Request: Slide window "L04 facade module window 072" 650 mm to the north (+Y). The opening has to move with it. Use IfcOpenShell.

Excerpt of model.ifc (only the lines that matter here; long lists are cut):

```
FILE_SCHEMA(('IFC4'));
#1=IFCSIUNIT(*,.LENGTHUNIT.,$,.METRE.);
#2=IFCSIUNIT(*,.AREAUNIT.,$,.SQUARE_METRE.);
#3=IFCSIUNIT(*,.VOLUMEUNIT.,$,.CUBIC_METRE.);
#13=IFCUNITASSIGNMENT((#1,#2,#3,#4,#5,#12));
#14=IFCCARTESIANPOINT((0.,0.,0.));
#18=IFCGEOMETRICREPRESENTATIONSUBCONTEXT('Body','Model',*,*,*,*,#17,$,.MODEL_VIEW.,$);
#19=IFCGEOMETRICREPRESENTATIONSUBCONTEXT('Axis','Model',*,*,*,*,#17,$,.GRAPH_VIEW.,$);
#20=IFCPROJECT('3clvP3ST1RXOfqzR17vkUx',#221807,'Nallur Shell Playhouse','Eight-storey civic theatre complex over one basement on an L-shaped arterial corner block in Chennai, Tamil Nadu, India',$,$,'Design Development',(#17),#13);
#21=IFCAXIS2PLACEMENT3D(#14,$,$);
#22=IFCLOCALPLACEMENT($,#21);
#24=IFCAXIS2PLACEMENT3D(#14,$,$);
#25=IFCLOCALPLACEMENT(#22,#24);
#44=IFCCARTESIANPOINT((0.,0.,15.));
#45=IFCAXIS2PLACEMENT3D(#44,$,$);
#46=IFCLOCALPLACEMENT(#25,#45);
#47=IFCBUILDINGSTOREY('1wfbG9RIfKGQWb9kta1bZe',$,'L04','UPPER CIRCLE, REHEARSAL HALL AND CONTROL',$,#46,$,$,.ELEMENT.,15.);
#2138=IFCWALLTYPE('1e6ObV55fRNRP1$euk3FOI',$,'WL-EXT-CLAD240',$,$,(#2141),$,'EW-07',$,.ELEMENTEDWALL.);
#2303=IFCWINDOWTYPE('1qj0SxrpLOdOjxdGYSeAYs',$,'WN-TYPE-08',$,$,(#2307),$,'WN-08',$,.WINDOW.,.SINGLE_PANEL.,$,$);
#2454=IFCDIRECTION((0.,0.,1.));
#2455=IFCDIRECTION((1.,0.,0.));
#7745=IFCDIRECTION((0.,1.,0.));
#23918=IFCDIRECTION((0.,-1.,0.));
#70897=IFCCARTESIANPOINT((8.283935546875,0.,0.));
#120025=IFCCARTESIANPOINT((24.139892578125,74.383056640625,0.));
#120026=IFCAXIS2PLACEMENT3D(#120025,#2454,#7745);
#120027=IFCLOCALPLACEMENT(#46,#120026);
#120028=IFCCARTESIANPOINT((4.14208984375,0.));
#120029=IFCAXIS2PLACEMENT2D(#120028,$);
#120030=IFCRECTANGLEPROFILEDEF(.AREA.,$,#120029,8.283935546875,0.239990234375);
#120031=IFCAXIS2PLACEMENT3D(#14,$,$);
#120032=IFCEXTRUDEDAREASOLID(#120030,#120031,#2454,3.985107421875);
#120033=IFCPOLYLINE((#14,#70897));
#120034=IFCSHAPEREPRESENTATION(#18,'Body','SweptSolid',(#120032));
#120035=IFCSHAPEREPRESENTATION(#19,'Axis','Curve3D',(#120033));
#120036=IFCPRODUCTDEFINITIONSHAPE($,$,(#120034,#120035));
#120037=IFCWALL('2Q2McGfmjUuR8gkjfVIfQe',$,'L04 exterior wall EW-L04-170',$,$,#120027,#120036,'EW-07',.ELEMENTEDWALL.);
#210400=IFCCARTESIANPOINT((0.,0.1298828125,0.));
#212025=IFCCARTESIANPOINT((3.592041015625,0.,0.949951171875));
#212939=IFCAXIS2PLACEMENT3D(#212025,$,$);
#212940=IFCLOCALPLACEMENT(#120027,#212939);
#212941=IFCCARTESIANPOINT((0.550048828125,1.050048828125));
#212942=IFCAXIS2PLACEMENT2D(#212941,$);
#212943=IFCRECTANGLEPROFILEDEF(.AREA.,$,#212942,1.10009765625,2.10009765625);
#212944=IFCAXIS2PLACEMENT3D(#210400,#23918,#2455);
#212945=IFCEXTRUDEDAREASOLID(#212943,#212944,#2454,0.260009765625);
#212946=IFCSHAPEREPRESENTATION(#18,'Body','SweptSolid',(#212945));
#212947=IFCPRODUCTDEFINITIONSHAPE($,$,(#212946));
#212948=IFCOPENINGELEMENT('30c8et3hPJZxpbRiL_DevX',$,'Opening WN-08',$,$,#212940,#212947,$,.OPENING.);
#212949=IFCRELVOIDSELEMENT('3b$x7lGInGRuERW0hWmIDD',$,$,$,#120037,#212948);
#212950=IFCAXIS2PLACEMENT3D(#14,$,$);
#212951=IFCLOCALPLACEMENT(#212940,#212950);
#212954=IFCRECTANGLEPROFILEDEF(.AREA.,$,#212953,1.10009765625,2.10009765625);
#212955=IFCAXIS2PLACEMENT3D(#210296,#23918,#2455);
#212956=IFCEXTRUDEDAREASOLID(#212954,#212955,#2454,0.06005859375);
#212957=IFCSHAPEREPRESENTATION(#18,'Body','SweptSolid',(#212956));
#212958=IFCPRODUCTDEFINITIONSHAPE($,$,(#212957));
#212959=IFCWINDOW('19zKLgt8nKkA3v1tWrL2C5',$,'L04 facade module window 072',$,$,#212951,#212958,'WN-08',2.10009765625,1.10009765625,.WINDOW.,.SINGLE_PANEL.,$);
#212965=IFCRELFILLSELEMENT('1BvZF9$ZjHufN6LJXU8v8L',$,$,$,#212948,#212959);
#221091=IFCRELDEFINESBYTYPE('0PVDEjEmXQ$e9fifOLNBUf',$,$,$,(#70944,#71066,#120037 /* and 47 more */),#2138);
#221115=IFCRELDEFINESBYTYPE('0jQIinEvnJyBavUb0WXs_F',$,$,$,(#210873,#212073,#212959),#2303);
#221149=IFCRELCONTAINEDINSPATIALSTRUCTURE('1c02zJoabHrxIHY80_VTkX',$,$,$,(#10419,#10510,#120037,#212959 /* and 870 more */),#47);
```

```python
import ifcopenshell
import ifcopenshell.api.geometry
import ifcopenshell.util.placement

model = ifcopenshell.open("model.ifc")

window = model.by_id(212959)
opening = window.FillsVoids[0].RelatingOpeningElement
wall = opening.VoidsElements[0].RelatingBuildingElement

wall_matrix = ifcopenshell.util.placement.get_local_placement(wall.ObjectPlacement)
shift = wall_matrix[:3, 0] * 0.65
before = ifcopenshell.util.placement.get_local_placement(window.ObjectPlacement)[:3, 3].copy()

# The window is placed relative to its opening, so it follows when the opening moves.
matrix = ifcopenshell.util.placement.get_local_placement(opening.ObjectPlacement)
matrix[:3, 3] += shift
ifcopenshell.api.geometry.edit_object_placement(
    model, product=opening, matrix=matrix, is_si=False, should_transform_children=True
)

after = ifcopenshell.util.placement.get_local_placement(window.ObjectPlacement)[:3, 3]
print("window moved by", (after - before).round(3) + 0.0)

model.write("model_v2.ifc")
```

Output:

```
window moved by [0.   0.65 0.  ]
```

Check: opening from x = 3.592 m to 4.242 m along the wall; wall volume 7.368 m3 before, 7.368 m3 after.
